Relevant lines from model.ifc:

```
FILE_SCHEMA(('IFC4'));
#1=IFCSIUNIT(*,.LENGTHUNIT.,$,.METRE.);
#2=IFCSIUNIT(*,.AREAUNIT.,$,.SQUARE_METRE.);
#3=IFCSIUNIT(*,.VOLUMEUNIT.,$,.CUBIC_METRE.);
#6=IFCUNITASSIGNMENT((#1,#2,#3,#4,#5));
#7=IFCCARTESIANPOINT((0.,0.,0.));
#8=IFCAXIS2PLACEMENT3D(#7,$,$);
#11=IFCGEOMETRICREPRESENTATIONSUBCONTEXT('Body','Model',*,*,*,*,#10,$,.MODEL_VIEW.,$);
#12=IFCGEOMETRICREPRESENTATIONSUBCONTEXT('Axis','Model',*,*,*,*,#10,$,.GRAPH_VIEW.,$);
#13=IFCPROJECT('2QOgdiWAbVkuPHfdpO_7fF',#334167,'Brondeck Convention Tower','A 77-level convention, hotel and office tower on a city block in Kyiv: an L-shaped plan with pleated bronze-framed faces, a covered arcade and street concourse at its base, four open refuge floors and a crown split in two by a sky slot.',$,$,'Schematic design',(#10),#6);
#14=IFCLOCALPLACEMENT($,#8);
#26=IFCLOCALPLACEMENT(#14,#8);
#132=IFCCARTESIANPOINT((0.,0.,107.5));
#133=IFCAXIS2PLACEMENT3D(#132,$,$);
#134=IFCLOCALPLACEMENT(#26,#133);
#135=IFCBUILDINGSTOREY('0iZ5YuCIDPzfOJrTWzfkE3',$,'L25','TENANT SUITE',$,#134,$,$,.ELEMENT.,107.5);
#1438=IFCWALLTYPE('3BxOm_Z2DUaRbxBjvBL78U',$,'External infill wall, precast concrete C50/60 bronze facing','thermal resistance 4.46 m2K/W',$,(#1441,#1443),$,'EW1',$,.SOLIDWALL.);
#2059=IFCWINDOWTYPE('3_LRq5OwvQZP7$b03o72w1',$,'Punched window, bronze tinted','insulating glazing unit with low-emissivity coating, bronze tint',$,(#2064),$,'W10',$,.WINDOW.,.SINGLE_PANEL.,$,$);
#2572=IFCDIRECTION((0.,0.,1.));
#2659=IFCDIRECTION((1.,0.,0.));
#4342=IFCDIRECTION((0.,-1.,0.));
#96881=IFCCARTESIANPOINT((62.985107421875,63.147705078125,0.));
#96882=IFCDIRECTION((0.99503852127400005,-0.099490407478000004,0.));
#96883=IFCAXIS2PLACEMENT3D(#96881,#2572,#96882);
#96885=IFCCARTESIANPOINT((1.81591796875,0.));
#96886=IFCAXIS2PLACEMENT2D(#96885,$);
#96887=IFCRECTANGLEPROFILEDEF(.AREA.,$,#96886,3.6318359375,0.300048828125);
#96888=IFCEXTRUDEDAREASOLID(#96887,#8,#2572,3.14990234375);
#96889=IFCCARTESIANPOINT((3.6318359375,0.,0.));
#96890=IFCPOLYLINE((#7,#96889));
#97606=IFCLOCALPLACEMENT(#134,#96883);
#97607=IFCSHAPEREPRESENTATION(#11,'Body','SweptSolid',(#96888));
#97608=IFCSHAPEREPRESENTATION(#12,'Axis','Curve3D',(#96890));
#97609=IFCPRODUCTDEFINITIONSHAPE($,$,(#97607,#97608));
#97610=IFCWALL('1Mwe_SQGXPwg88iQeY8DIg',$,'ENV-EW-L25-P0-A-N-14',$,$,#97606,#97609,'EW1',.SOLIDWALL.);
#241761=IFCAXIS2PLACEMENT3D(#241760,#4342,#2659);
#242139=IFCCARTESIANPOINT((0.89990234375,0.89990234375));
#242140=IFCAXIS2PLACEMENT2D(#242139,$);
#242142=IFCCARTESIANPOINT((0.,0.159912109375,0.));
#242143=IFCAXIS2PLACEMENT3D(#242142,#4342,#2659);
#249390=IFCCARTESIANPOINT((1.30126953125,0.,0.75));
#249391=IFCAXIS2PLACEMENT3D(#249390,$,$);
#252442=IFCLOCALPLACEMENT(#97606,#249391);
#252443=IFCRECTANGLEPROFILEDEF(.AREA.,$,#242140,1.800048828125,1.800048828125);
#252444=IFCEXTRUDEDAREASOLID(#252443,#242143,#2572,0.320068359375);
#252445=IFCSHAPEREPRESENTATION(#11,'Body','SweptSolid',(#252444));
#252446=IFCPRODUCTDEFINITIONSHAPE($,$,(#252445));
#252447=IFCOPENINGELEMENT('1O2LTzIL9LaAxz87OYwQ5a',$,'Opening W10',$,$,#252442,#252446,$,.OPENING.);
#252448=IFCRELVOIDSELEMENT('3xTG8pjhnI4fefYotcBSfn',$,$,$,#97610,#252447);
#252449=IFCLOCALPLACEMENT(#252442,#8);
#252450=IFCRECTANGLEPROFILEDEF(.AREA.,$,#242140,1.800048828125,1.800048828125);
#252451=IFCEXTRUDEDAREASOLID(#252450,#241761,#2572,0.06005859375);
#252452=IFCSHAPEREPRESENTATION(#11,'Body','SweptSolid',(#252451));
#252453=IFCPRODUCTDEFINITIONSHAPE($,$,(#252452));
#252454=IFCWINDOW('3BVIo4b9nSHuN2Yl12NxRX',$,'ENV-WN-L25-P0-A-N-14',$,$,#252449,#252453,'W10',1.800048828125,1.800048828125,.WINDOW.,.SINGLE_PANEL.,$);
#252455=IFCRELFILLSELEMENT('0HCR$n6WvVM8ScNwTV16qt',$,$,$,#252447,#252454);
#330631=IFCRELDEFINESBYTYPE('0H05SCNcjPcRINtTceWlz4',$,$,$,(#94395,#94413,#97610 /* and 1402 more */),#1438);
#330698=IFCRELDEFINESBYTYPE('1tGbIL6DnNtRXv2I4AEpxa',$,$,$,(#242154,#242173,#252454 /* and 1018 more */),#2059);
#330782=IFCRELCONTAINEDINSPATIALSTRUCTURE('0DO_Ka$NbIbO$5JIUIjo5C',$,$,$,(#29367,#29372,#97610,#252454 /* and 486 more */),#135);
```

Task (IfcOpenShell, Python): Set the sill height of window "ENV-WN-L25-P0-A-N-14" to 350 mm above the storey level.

```python
import numpy as np
import ifcopenshell
import ifcopenshell.api.geometry
import ifcopenshell.geom
import ifcopenshell.util.element
import ifcopenshell.util.placement
import ifcopenshell.util.shape
import ifcopenshell.util.unit

model = ifcopenshell.open("model.ifc")
unit_scale = ifcopenshell.util.unit.calculate_unit_scale(model)

window = model.by_guid("3BVIo4b9nSHuN2Yl12NxRX")
opening = window.FillsVoids[0].RelatingOpeningElement
storey = ifcopenshell.util.element.get_container(window, ifc_class="IfcBuildingStorey")
level = ifcopenshell.util.placement.get_local_placement(storey.ObjectPlacement)[2, 3]

# The opening's origin need not be at the sill, so measure its lowest point.
shape = ifcopenshell.geom.create_shape(ifcopenshell.geom.settings(), opening)
bottom = ifcopenshell.util.shape.get_shape_bottom_elevation(shape, shape.geometry) / unit_scale
dz = level + 0.35 / unit_scale - bottom

shift = np.array([0.0, 0.0, dz])
# The window is placed relative to its opening, so it follows when the opening moves.
matrix = ifcopenshell.util.placement.get_local_placement(opening.ObjectPlacement)
matrix[:3, 3] += shift
ifcopenshell.api.geometry.edit_object_placement(
    model, product=opening, matrix=matrix, is_si=False, should_transform_children=True
)

print(f"moved by {dz * unit_scale:+.3f} m")

model.write("model_edited.ifc")
```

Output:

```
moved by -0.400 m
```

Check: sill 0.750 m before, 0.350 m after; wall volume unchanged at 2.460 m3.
